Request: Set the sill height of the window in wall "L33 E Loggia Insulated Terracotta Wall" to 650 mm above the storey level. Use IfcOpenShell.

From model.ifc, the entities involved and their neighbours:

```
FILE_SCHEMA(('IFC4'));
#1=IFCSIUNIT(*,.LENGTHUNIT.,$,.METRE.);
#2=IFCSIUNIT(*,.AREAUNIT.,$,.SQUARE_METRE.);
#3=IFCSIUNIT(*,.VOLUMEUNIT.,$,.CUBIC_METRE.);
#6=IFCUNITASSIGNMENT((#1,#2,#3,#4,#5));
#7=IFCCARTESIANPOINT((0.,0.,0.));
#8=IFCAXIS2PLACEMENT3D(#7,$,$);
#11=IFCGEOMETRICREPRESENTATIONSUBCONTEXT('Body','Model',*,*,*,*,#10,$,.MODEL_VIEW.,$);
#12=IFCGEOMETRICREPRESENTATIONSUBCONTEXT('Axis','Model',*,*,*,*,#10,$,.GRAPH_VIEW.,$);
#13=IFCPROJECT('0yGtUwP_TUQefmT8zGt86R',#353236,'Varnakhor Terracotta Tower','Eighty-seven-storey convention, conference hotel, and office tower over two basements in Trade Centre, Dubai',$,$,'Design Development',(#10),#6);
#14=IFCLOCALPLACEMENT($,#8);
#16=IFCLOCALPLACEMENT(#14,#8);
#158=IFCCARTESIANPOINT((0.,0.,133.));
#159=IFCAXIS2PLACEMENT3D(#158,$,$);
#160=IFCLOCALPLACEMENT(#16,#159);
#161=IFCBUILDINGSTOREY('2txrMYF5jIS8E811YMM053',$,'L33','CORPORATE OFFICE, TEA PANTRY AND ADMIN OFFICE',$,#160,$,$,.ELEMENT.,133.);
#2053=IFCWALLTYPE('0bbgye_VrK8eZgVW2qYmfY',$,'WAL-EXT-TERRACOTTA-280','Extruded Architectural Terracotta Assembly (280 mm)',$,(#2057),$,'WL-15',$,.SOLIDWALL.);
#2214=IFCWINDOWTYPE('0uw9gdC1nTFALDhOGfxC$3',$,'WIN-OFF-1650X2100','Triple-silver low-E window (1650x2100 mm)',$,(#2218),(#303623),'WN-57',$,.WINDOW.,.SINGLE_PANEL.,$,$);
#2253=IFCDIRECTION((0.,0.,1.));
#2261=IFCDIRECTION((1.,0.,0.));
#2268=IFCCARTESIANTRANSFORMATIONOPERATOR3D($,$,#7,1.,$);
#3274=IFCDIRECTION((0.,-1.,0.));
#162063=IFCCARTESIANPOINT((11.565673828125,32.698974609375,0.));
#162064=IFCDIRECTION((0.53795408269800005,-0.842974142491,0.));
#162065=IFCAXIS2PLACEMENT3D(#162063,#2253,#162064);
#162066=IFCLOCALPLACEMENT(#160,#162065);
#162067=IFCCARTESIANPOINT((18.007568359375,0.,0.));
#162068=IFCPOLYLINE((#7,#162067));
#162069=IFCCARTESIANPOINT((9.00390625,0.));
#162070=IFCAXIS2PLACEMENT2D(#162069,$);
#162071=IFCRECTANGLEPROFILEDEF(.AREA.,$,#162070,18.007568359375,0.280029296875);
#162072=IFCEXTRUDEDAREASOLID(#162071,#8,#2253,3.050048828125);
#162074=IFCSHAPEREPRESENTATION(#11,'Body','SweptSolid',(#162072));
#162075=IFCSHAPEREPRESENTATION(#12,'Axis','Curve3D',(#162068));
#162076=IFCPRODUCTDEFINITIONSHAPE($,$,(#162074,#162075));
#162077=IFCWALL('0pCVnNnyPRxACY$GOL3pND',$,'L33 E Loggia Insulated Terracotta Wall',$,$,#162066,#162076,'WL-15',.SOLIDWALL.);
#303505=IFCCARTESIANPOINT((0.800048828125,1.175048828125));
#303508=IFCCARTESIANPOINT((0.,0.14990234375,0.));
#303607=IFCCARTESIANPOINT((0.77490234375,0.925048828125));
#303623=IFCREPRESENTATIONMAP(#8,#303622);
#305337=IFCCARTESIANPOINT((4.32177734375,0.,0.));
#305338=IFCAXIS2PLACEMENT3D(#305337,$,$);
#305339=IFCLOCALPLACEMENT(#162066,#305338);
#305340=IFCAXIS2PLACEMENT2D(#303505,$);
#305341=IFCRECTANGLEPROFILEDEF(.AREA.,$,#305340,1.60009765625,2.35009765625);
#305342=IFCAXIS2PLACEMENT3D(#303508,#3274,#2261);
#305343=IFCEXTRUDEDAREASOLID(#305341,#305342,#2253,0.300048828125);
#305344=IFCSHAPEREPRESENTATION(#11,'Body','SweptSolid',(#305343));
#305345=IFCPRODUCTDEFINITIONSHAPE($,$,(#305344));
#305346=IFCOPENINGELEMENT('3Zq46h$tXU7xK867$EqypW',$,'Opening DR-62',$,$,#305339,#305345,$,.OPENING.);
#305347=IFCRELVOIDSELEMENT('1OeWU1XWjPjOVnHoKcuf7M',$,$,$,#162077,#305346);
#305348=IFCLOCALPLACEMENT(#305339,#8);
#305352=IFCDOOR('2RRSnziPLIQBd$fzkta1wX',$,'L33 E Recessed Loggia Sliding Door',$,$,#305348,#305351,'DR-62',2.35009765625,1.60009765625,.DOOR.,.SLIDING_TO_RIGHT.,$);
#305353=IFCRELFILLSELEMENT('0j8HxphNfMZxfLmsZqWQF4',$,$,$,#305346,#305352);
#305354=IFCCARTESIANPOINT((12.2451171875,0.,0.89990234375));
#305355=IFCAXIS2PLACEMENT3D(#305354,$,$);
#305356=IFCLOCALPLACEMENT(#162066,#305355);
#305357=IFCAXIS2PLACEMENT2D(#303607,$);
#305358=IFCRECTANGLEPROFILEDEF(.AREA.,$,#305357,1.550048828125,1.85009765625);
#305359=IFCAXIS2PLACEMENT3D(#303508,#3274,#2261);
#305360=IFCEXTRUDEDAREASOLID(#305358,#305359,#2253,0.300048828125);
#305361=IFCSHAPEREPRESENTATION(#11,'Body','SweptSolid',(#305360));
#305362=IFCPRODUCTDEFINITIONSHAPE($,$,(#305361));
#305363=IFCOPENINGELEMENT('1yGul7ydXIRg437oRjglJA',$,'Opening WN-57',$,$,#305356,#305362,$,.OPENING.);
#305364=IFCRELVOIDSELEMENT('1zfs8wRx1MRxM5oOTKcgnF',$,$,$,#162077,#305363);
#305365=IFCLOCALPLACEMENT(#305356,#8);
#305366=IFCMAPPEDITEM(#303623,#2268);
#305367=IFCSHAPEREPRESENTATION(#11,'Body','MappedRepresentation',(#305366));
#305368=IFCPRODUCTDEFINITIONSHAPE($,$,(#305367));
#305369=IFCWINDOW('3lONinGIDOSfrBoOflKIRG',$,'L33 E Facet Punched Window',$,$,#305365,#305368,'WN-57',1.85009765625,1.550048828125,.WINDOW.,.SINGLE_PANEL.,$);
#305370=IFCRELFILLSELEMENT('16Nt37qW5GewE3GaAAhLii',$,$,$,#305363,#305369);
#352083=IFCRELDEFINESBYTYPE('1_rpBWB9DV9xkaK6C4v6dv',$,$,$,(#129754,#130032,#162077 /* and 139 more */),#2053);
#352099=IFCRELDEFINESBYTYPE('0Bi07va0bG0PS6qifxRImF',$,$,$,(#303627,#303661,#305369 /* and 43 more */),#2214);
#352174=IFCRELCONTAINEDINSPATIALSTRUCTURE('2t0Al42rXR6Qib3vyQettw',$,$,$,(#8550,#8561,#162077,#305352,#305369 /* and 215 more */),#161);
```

```python
import numpy as np
import ifcopenshell
import ifcopenshell.api.geometry
import ifcopenshell.geom
import ifcopenshell.util.element
import ifcopenshell.util.placement
import ifcopenshell.util.shape
import ifcopenshell.util.unit

model = ifcopenshell.open("model.ifc")
unit_scale = ifcopenshell.util.unit.calculate_unit_scale(model)

window = model.by_id(305369)
opening = window.FillsVoids[0].RelatingOpeningElement
storey = ifcopenshell.util.element.get_container(window, ifc_class="IfcBuildingStorey")
level = ifcopenshell.util.placement.get_local_placement(storey.ObjectPlacement)[2, 3]

# The opening's origin need not be at the sill, so measure its lowest point.
shape = ifcopenshell.geom.create_shape(ifcopenshell.geom.settings(), opening)
bottom = ifcopenshell.util.shape.get_shape_bottom_elevation(shape, shape.geometry) / unit_scale
dz = level + 0.65 - bottom

shift = np.array([0.0, 0.0, dz])
# The window is placed relative to its opening, so it follows when the opening moves.
matrix = ifcopenshell.util.placement.get_local_placement(opening.ObjectPlacement)
matrix[:3, 3] += shift
ifcopenshell.api.geometry.edit_object_placement(
    model, product=opening, matrix=matrix, is_si=False, should_transform_children=True
)

print(f"moved by {dz * unit_scale:+.3f} m")

model.write("model_edited.ifc")
```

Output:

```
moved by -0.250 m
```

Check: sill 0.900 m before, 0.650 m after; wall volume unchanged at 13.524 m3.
